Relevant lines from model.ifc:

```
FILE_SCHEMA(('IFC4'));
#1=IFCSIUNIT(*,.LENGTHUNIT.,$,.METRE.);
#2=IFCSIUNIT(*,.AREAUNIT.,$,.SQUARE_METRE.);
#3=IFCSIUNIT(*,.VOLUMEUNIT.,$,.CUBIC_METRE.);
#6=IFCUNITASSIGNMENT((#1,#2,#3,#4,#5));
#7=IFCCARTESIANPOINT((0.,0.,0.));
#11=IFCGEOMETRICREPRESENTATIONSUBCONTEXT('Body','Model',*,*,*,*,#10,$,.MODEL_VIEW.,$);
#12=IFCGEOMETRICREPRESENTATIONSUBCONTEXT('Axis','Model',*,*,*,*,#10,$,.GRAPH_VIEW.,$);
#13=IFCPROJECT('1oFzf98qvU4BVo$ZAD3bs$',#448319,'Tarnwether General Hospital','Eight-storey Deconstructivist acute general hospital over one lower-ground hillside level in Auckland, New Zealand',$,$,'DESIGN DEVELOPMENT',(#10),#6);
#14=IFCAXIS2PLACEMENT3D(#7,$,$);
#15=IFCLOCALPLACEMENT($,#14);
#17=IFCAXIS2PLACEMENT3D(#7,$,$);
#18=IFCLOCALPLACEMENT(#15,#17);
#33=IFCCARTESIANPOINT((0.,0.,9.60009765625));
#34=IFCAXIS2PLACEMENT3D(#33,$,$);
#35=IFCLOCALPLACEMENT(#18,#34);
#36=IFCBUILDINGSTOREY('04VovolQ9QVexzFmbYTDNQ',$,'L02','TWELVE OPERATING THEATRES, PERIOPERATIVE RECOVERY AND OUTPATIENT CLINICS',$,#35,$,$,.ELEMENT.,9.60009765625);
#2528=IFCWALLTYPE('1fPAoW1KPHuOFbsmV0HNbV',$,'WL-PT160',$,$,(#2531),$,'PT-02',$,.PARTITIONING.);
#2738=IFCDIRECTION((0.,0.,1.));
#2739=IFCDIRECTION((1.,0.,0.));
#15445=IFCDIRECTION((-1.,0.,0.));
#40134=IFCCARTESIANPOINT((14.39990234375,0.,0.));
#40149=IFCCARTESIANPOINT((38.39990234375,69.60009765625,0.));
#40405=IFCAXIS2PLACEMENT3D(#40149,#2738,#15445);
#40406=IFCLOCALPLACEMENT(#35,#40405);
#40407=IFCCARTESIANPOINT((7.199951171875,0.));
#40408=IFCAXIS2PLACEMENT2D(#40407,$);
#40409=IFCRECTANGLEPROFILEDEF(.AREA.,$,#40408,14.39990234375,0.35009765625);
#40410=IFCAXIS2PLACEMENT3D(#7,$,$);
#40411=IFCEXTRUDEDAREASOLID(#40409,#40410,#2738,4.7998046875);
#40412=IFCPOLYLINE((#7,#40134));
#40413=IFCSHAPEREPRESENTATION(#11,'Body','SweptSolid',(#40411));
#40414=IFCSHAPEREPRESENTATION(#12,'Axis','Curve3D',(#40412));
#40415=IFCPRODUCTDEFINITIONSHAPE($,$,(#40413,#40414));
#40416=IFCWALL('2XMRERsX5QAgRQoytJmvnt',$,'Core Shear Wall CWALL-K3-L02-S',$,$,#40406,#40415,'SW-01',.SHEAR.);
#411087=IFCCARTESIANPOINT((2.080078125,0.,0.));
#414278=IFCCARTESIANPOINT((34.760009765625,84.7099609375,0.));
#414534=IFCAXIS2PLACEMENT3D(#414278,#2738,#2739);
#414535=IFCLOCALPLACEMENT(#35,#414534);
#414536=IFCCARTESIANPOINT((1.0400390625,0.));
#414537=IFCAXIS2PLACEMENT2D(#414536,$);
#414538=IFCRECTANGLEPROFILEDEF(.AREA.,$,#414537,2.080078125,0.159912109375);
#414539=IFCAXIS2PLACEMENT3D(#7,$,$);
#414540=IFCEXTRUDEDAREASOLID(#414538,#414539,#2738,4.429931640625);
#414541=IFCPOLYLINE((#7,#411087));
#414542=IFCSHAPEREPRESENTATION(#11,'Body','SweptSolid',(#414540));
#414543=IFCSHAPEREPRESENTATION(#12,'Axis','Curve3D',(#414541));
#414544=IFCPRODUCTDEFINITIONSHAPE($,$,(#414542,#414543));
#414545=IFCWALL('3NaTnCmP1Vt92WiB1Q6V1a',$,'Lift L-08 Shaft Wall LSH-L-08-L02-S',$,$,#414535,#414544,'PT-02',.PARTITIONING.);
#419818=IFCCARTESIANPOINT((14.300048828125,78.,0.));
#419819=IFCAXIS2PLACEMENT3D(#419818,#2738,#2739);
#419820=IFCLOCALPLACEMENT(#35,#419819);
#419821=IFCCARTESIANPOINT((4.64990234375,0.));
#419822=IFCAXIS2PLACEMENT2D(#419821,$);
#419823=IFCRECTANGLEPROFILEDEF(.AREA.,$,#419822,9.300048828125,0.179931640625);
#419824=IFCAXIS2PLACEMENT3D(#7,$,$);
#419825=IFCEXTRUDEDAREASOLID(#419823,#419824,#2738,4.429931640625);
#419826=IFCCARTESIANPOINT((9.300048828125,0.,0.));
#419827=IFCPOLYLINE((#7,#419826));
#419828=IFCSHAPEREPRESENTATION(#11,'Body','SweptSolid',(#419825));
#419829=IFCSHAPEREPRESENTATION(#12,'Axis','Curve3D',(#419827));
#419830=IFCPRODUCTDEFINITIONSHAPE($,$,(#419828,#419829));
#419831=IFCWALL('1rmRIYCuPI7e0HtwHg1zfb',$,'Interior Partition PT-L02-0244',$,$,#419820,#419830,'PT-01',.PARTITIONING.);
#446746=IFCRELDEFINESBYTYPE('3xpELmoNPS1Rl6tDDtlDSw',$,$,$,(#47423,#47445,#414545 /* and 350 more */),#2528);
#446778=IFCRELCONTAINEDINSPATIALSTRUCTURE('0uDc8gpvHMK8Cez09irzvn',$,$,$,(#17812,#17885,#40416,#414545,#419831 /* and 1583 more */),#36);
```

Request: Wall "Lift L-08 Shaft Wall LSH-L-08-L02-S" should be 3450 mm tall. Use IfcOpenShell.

```python
import ifcopenshell
import ifcopenshell.geom
import ifcopenshell.util.representation
import ifcopenshell.util.shape

model = ifcopenshell.open("model.ifc")
settings = ifcopenshell.geom.settings()


def volume(element):
    """Net volume in cubic metres, openings subtracted."""
    shape = ifcopenshell.geom.create_shape(settings, element)
    return ifcopenshell.util.shape.get_volume(shape.geometry)


wall = model.by_guid("3NaTnCmP1Vt92WiB1Q6V1a")
before = volume(wall)

body = ifcopenshell.util.representation.get_representation(wall, "Model", "Body")
solid = body.Items[0]
old_height = solid.Depth
solid.Depth = 3.45
after = volume(wall)

print(f"height {old_height:g} -> {solid.Depth:g}, volume {before:.3f} -> {after:.3f} m3")

model.write("model-out.ifc")
```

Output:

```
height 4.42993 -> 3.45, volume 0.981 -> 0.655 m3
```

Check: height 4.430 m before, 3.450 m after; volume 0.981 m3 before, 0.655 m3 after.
